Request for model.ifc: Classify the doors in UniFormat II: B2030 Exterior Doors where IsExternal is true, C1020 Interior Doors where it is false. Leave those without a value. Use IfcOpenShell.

First a look at what the model holds.

```python
import ifcopenshell
import ifcopenshell.util.element

model = ifcopenshell.open("model.ifc")
print(model.schema)
print("classifications:", [c.Name for c in model.by_type("IfcClassification")])
values = [ifcopenshell.util.element.get_pset(e, "Pset_DoorCommon", "IsExternal") for e in model.by_type("IfcDoor")]
for value in (True, False, None):
    print("IsExternal", value, values.count(value))
```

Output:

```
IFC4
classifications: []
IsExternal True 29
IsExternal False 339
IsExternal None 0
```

```python
import ifcopenshell
import ifcopenshell.api.classification
import ifcopenshell.util.element

model = ifcopenshell.open("model.ifc")

system = ifcopenshell.api.classification.add_classification(model, classification="UniFormat II")

doors = model.by_type("IfcDoor")
external = {e: ifcopenshell.util.element.get_pset(e, "Pset_DoorCommon", "IsExternal") for e in doors}
for flag, code, name in ((True, "B2030", "Exterior Doors"), (False, "C1020", "Interior Doors")):
    products = [e for e in doors if external[e] is flag]
    ifcopenshell.api.classification.add_reference(
        model, products=products, classification=system, identification=code, name=name
    )
    print(code, len(products))

model.write("model_v2.ifc")
```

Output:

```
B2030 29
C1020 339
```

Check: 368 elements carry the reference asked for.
